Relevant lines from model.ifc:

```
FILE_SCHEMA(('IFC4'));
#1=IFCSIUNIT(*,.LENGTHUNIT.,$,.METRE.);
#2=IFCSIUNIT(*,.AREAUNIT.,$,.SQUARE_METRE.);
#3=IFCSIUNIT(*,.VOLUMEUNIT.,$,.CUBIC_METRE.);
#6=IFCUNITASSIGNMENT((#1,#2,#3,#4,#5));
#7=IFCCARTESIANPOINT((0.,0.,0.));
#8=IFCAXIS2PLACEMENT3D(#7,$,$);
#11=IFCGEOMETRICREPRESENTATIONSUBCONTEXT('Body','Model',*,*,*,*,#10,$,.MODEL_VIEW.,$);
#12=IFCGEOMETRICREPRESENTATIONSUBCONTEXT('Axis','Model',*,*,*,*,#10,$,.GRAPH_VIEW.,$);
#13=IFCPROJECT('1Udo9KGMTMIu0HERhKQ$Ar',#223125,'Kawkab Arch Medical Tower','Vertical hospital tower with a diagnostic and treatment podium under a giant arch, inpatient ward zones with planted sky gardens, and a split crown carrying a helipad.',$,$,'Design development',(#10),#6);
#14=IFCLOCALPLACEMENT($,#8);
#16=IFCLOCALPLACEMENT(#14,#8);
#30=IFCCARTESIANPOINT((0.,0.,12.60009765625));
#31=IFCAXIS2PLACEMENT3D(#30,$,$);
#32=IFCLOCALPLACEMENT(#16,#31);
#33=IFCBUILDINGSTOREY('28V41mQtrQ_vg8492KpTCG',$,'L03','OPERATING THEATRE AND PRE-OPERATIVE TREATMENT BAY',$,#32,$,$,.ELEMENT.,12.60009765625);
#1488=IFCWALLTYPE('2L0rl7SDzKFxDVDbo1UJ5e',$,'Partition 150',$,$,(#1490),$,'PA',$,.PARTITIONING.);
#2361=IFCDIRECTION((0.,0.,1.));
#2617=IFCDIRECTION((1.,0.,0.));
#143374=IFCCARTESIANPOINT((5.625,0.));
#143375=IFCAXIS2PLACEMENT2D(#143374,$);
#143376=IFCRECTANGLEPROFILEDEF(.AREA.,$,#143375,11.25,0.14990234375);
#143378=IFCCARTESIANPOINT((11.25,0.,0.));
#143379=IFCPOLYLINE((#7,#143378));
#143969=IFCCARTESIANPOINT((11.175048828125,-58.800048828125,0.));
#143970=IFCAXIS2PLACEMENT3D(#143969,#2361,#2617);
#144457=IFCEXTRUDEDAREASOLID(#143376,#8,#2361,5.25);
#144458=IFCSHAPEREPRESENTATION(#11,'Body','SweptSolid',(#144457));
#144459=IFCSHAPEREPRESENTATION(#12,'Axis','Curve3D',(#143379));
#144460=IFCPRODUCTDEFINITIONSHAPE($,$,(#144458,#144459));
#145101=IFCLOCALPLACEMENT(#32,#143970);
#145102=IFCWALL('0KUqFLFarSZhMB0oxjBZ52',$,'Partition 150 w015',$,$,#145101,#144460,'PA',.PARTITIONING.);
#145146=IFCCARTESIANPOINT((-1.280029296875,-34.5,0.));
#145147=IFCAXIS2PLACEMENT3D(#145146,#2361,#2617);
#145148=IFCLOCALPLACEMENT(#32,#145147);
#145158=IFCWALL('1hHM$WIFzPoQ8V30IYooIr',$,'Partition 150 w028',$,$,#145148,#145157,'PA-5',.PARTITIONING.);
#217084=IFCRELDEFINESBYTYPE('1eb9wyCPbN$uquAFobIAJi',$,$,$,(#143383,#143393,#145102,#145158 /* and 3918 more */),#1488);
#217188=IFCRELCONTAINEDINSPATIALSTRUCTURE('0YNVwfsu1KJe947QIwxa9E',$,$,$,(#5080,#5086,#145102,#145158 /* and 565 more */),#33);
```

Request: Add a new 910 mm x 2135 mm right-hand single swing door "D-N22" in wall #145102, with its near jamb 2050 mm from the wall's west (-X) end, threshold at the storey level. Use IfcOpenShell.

```python
import numpy as np
import ifcopenshell
import ifcopenshell.api.feature
import ifcopenshell.api.geometry
import ifcopenshell.api.root
import ifcopenshell.api.spatial
import ifcopenshell.geom
import ifcopenshell.util.element
import ifcopenshell.util.placement
import ifcopenshell.util.representation
import ifcopenshell.util.shape
import ifcopenshell.util.unit

model = ifcopenshell.open("model.ifc")
unit_scale = ifcopenshell.util.unit.calculate_unit_scale(model)
settings = ifcopenshell.geom.settings()


def volume(element):
    """Net volume in cubic metres, openings subtracted."""
    shape = ifcopenshell.geom.create_shape(settings, element)
    return ifcopenshell.util.shape.get_volume(shape.geometry)


wall = model.by_guid("0KUqFLFarSZhMB0oxjBZ52")
storey = ifcopenshell.util.element.get_container(wall, ifc_class="IfcBuildingStorey")
context = ifcopenshell.util.representation.get_context(model, "Model", "Body", "MODEL_VIEW")
before = volume(wall)

width, height, from_end, sill = 0.91, 2.135, 2.05, 0.0  # metres

# The wall runs along its own X axis, and the end named is its -X end.
wall_shape = ifcopenshell.geom.create_shape(settings, wall)
x, y, z = ifcopenshell.util.shape.get_vertices(wall_shape.geometry).T
start = x.min() + from_end
face, thickness = float(y.min()), float(y.max() - y.min())
wall_matrix = ifcopenshell.util.placement.get_local_placement(wall.ObjectPlacement)
level = ifcopenshell.util.placement.get_local_placement(storey.ObjectPlacement)[2, 3]


def in_wall(x, y):
    """Placement at x, y metres in the wall's axes, at sill height."""
    matrix = wall_matrix.copy()
    matrix[:, 3] = wall_matrix @ np.array([x / unit_scale, y / unit_scale, 0.0, 1.0])
    matrix[2, 3] = level + sill / unit_scale
    return matrix


# Opening: a box that overshoots both wall faces by 50 mm.
opening = ifcopenshell.api.root.create_entity(model, ifc_class="IfcOpeningElement", predefined_type="OPENING")
box = ifcopenshell.api.geometry.add_wall_representation(
    model, context=context, length=width, height=height, thickness=thickness + 0.1
)
ifcopenshell.api.geometry.assign_representation(model, product=opening, representation=box)
ifcopenshell.api.geometry.edit_object_placement(model, product=opening, matrix=in_wall(start, face - 0.05), is_si=False)
ifcopenshell.api.feature.add_feature(model, feature=opening, element=wall)

door = ifcopenshell.api.root.create_entity(model, ifc_class="IfcDoor", name="D-N22", predefined_type="DOOR")
door.OverallWidth, door.OverallHeight = width / unit_scale, height / unit_scale
door.OperationType = "SINGLE_SWING_RIGHT"
body = ifcopenshell.api.geometry.add_door_representation(
    model,
    context=context,
    overall_width=door.OverallWidth,
    overall_height=door.OverallHeight,
    operation_type="SINGLE_SWING_RIGHT",
    lining_properties={"LiningDepth": thickness / unit_scale, "ThresholdDepth": thickness / unit_scale},
)
ifcopenshell.api.geometry.assign_representation(model, product=door, representation=body)
ifcopenshell.api.spatial.assign_container(model, products=[door], relating_structure=storey)
ifcopenshell.api.feature.add_filling(model, opening=opening, element=door)

# The lining spans the wall, so the door starts at the wall face.
ifcopenshell.api.geometry.edit_object_placement(model, product=door, matrix=in_wall(start, face), is_si=False)

after = volume(wall)

print(f"wall volume {before:.3f} -> {after:.3f} m3")

model.write("model-out.ifc")
```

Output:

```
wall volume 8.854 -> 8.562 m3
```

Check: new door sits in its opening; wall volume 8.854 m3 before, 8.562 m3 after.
